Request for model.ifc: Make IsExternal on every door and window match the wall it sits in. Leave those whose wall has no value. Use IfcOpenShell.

First a look at what the model holds.

```python
import ifcopenshell
import ifcopenshell.util.element

model = ifcopenshell.open("model.ifc")
print(model.schema)
seen = {}
for e in model.by_type("IfcDoor") + model.by_type("IfcWindow"):
    if not e.FillsVoids:
        continue
    host = e.FillsVoids[0].RelatingOpeningElement.VoidsElements[0].RelatingBuildingElement
    own = ifcopenshell.util.element.get_pset(e, f"Pset_{e.is_a()[3:].removesuffix('StandardCase')}Common", "IsExternal")
    wall = ifcopenshell.util.element.get_pset(host, "Pset_WallCommon", "IsExternal")
    seen[e.is_a(), own, wall] = seen.get((e.is_a(), own, wall), 0) + 1
for (cls, own, wall), count in sorted(seen.items(), key=str):
    print(count, cls, "IsExternal:", own, "| host wall:", wall)
```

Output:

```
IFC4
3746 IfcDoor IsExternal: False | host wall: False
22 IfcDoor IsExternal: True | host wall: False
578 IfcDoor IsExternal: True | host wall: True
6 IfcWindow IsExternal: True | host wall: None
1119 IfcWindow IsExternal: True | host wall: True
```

```python
import ifcopenshell
import ifcopenshell.api.pset
import ifcopenshell.util.element

model = ifcopenshell.open("model.ifc")

count = 0
for ifc_class, pset_name in (("IfcDoor", "Pset_DoorCommon"), ("IfcWindow", "Pset_WindowCommon")):
    for e in model.by_type(ifc_class):
        if not e.FillsVoids:
            continue
        host = e.FillsVoids[0].RelatingOpeningElement.VoidsElements[0].RelatingBuildingElement
        external = ifcopenshell.util.element.get_pset(host, "Pset_WallCommon", "IsExternal")
        if external is None or ifcopenshell.util.element.get_pset(e, pset_name, "IsExternal") == external:
            continue
        pset = ifcopenshell.api.pset.add_pset(model, product=e, name=pset_name)
        ifcopenshell.api.pset.edit_pset(model, pset=pset, properties={"IsExternal": external})
        count += 1

print(count, "updated")

model.write("model_v2.ifc")
```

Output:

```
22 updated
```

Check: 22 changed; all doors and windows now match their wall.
